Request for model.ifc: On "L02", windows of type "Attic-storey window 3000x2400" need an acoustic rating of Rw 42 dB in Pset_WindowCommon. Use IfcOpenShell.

First a look at what the model holds.

```python
import ifcopenshell
import ifcopenshell.util.element

model = ifcopenshell.open("model.ifc")
print(model.schema)
storey = next(s for s in model.by_type("IfcBuildingStorey") if s.Name == "L02")
windows = [e for e in ifcopenshell.util.element.get_decomposition(storey) if e.is_a("IfcWindow")]
seen = {}
for e in windows:
    element_type = ifcopenshell.util.element.get_type(e)
    key = (element_type.Name if element_type != e and element_type else None, ifcopenshell.util.element.get_pset(e, "Pset_WindowCommon", "AcousticRating"))
    seen[key] = seen.get(key, 0) + 1
for (name, value), count in sorted(seen.items(), key=str):
    print(count, "x", name, "|", value)
```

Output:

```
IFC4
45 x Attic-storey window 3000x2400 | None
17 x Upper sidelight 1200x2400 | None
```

```python
import ifcopenshell
import ifcopenshell.api.pset
import ifcopenshell.util.element

model = ifcopenshell.open("model.ifc")

storey = next(s for s in model.by_type("IfcBuildingStorey") if s.Name == "L02")
windows = [e for e in ifcopenshell.util.element.get_decomposition(storey) if e.is_a("IfcWindow")]

count = 0
for e in windows:
    element_type = ifcopenshell.util.element.get_type(e)
    if element_type in (None, e) or element_type.Name != "Attic-storey window 3000x2400":
        continue
    # add_pset returns the element's existing set when there is one.
    pset = ifcopenshell.api.pset.add_pset(model, product=e, name="Pset_WindowCommon")
    ifcopenshell.api.pset.edit_pset(model, pset=pset, properties={"AcousticRating": "Rw 42 dB"})
    count += 1

print(count, "windows updated")

model.write("model-out.ifc")
```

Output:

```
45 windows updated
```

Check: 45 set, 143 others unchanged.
